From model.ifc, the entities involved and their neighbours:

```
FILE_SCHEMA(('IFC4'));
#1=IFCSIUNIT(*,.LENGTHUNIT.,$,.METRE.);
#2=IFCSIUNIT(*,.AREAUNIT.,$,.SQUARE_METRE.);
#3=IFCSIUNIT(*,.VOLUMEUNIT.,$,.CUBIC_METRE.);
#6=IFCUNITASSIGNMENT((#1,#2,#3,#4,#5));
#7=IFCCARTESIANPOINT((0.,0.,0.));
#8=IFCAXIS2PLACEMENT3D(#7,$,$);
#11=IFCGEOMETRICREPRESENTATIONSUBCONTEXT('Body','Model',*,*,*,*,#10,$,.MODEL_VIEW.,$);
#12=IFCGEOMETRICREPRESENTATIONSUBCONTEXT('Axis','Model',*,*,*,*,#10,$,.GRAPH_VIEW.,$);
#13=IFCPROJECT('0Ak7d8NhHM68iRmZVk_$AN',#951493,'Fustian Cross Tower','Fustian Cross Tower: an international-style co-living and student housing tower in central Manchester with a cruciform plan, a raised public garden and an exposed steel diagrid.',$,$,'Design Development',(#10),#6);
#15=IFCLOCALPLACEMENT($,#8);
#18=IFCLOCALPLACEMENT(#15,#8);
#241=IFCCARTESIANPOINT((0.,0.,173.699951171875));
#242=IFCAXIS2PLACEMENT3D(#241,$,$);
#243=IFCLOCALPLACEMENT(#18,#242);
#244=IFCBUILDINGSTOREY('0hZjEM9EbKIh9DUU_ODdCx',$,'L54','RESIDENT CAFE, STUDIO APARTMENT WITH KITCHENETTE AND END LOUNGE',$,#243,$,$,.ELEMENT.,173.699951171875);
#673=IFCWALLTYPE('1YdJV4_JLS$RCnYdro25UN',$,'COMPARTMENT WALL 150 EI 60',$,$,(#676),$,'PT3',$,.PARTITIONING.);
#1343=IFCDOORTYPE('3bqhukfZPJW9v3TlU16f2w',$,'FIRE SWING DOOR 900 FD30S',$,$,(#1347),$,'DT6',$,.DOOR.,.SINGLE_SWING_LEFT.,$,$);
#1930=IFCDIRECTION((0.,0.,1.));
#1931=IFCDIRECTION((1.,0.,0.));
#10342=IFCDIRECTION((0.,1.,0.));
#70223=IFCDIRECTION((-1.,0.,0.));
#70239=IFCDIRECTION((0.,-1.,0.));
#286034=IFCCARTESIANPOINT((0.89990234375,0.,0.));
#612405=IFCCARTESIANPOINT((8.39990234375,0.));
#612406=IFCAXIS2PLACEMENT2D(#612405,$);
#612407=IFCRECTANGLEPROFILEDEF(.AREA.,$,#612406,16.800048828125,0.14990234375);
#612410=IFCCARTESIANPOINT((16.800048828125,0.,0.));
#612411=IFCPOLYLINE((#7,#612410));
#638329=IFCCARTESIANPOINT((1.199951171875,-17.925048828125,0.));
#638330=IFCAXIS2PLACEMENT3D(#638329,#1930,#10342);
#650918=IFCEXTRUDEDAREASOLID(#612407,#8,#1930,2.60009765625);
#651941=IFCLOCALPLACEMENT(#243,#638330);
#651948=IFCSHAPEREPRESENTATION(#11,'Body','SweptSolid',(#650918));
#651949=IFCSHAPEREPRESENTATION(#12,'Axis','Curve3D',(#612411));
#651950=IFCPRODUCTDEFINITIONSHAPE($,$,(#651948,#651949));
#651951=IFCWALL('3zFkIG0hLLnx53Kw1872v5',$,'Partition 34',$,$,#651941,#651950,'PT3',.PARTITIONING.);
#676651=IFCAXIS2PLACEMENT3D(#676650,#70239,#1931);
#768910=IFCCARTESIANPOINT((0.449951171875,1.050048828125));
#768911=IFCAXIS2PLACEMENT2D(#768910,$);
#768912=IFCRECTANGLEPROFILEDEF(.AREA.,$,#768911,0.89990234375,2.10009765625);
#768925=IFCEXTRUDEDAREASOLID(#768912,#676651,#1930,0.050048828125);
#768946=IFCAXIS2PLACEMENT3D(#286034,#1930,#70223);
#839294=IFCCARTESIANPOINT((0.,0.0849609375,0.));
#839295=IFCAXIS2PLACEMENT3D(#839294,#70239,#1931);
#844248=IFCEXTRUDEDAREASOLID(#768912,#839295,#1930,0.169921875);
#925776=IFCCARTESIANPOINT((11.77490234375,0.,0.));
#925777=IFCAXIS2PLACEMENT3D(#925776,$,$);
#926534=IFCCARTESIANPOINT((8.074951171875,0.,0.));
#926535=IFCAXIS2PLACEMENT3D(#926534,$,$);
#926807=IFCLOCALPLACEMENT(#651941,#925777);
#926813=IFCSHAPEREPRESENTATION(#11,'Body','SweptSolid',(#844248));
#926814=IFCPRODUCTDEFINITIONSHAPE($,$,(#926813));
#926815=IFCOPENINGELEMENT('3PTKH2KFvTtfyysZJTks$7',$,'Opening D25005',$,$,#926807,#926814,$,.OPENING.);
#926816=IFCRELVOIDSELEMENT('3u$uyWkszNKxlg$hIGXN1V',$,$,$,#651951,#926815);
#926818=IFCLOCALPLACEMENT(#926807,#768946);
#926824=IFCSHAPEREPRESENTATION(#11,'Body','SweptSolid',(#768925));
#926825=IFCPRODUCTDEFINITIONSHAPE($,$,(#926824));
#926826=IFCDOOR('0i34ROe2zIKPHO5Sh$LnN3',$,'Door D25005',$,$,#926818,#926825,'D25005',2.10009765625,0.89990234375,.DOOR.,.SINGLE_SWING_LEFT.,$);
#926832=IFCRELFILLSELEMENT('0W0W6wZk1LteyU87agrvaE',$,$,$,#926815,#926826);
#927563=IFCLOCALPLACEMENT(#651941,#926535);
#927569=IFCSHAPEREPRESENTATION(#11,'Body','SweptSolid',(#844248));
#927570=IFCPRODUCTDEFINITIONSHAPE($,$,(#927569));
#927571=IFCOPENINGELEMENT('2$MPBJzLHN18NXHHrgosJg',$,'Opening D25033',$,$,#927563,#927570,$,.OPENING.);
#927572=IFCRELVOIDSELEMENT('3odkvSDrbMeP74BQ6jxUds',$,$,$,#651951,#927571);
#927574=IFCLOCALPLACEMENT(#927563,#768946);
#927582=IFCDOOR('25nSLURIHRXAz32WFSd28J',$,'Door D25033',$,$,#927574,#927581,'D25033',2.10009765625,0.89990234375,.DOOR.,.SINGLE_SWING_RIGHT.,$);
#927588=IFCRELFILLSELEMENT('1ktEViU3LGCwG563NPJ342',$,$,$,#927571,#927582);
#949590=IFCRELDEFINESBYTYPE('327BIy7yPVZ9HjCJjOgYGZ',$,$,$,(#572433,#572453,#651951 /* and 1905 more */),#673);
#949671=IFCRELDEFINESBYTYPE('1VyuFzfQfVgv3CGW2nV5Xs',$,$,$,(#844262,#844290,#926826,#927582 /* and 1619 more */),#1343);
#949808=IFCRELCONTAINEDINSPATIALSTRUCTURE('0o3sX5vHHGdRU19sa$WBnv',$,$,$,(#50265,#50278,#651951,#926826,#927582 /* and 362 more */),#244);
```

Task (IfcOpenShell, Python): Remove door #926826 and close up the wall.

```python
import ifcopenshell
import ifcopenshell.api.feature
import ifcopenshell.api.root
import ifcopenshell.geom
import ifcopenshell.util.shape

model = ifcopenshell.open("model.ifc")
settings = ifcopenshell.geom.settings()


def volume(element):
    """Net volume in cubic metres, openings subtracted."""
    shape = ifcopenshell.geom.create_shape(settings, element)
    return ifcopenshell.util.shape.get_volume(shape.geometry)


door = model.by_guid("0i34ROe2zIKPHO5Sh$LnN3")
opening = door.FillsVoids[0].RelatingOpeningElement
wall = opening.VoidsElements[0].RelatingBuildingElement
before = volume(wall)

ifcopenshell.api.root.remove_product(model, product=door)
ifcopenshell.api.feature.remove_feature(model, feature=opening)

after = volume(wall)

print(f"wall volume {before:.3f} -> {after:.3f} m3")

model.write("model_updated.ifc")
```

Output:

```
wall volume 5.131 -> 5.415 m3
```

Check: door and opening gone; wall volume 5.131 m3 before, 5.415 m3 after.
